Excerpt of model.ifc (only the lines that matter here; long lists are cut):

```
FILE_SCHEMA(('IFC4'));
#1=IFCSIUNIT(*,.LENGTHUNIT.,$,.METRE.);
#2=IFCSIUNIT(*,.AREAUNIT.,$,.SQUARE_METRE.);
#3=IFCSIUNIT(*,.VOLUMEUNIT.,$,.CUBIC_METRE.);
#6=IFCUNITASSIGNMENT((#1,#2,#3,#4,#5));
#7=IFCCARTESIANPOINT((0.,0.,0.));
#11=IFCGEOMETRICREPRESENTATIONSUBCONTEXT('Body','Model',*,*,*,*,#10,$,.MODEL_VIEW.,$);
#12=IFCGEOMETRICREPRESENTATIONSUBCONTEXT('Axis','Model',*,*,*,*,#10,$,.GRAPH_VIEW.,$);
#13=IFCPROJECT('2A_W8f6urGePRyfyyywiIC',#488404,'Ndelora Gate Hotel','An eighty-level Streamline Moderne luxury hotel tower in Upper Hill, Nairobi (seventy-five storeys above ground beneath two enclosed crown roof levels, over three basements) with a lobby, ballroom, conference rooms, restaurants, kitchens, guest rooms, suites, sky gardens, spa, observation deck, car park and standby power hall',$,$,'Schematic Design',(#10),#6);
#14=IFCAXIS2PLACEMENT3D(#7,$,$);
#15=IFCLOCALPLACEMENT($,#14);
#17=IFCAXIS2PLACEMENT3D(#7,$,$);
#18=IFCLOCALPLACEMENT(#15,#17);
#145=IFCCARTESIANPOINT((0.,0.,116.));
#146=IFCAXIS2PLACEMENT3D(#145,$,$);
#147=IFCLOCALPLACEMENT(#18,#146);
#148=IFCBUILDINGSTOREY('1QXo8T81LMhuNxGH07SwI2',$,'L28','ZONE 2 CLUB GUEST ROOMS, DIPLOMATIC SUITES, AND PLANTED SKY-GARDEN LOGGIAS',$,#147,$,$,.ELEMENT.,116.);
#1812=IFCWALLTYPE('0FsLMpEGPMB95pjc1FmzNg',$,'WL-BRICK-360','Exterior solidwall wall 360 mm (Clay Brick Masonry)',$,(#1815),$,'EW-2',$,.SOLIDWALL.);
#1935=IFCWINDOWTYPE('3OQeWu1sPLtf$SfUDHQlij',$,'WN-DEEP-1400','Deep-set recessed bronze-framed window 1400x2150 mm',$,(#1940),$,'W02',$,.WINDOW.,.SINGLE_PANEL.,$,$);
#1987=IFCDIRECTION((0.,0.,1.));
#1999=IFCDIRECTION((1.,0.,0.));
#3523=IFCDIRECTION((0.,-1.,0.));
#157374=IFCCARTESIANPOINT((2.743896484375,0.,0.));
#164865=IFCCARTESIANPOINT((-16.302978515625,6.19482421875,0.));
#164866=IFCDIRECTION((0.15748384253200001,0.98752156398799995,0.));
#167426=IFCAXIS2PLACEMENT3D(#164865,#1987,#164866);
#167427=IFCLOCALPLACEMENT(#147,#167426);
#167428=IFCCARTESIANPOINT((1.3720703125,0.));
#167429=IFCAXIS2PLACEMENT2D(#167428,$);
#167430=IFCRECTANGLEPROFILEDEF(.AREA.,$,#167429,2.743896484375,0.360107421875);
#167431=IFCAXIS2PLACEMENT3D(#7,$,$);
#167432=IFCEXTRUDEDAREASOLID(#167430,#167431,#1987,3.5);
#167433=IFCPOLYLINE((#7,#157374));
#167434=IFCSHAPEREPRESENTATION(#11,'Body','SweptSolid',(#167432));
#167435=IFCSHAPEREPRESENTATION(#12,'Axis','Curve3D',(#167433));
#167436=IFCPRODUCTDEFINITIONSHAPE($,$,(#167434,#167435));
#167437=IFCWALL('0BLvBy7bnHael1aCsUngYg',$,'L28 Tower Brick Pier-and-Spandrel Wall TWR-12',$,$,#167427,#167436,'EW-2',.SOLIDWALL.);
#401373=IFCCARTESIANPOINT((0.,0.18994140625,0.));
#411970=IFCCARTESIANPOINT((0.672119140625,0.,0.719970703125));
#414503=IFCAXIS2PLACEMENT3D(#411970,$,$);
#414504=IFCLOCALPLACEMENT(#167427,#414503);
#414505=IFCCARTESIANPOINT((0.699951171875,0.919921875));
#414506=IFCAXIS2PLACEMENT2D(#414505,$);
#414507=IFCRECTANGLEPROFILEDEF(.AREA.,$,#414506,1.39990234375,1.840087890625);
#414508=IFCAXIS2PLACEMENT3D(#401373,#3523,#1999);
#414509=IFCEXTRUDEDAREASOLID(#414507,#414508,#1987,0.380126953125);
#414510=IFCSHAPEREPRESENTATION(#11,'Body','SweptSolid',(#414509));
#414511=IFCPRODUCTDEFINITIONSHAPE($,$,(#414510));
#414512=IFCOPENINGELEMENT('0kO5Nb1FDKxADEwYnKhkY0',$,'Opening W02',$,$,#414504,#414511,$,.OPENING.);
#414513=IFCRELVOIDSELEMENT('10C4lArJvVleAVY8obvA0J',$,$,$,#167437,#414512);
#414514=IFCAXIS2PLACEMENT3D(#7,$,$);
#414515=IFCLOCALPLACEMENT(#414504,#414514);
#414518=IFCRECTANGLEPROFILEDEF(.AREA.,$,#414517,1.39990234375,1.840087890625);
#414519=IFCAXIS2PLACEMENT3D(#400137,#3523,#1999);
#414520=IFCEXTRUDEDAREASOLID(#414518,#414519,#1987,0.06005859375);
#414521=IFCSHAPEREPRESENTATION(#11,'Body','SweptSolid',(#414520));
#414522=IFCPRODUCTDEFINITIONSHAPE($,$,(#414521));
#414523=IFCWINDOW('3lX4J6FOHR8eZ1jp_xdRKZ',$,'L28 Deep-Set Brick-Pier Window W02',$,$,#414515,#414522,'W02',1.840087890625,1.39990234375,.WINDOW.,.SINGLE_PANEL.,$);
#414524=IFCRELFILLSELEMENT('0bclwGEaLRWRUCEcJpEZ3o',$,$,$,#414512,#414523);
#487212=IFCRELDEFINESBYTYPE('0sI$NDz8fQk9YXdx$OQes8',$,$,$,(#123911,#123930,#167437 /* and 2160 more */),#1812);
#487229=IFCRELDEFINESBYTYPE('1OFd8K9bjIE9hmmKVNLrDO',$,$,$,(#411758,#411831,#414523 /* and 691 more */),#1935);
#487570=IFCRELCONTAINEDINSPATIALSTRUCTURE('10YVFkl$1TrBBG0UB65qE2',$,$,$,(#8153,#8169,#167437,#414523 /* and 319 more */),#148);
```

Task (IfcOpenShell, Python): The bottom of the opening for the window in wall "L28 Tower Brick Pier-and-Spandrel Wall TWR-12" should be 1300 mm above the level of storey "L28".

```python
import numpy as np
import ifcopenshell
import ifcopenshell.api.geometry
import ifcopenshell.geom
import ifcopenshell.util.element
import ifcopenshell.util.placement
import ifcopenshell.util.shape
import ifcopenshell.util.unit

model = ifcopenshell.open("model.ifc")
unit_scale = ifcopenshell.util.unit.calculate_unit_scale(model)

window = model.by_id(414523)
opening = window.FillsVoids[0].RelatingOpeningElement
storey = ifcopenshell.util.element.get_container(window, ifc_class="IfcBuildingStorey")
level = ifcopenshell.util.placement.get_local_placement(storey.ObjectPlacement)[2, 3]

# The opening's origin need not be at the sill, so measure its lowest point.
shape = ifcopenshell.geom.create_shape(ifcopenshell.geom.settings(), opening)
bottom = ifcopenshell.util.shape.get_shape_bottom_elevation(shape, shape.geometry) / unit_scale
dz = level + 1.3 / unit_scale - bottom

shift = np.array([0.0, 0.0, dz])
# The window is placed relative to its opening, so it follows when the opening moves.
matrix = ifcopenshell.util.placement.get_local_placement(opening.ObjectPlacement)
matrix[:3, 3] += shift
ifcopenshell.api.geometry.edit_object_placement(
    model, product=opening, matrix=matrix, is_si=False, should_transform_children=True
)

print(f"moved by {dz * unit_scale:+.3f} m")

model.write("model_updated.ifc")
```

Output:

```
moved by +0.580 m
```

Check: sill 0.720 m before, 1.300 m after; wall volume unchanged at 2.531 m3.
